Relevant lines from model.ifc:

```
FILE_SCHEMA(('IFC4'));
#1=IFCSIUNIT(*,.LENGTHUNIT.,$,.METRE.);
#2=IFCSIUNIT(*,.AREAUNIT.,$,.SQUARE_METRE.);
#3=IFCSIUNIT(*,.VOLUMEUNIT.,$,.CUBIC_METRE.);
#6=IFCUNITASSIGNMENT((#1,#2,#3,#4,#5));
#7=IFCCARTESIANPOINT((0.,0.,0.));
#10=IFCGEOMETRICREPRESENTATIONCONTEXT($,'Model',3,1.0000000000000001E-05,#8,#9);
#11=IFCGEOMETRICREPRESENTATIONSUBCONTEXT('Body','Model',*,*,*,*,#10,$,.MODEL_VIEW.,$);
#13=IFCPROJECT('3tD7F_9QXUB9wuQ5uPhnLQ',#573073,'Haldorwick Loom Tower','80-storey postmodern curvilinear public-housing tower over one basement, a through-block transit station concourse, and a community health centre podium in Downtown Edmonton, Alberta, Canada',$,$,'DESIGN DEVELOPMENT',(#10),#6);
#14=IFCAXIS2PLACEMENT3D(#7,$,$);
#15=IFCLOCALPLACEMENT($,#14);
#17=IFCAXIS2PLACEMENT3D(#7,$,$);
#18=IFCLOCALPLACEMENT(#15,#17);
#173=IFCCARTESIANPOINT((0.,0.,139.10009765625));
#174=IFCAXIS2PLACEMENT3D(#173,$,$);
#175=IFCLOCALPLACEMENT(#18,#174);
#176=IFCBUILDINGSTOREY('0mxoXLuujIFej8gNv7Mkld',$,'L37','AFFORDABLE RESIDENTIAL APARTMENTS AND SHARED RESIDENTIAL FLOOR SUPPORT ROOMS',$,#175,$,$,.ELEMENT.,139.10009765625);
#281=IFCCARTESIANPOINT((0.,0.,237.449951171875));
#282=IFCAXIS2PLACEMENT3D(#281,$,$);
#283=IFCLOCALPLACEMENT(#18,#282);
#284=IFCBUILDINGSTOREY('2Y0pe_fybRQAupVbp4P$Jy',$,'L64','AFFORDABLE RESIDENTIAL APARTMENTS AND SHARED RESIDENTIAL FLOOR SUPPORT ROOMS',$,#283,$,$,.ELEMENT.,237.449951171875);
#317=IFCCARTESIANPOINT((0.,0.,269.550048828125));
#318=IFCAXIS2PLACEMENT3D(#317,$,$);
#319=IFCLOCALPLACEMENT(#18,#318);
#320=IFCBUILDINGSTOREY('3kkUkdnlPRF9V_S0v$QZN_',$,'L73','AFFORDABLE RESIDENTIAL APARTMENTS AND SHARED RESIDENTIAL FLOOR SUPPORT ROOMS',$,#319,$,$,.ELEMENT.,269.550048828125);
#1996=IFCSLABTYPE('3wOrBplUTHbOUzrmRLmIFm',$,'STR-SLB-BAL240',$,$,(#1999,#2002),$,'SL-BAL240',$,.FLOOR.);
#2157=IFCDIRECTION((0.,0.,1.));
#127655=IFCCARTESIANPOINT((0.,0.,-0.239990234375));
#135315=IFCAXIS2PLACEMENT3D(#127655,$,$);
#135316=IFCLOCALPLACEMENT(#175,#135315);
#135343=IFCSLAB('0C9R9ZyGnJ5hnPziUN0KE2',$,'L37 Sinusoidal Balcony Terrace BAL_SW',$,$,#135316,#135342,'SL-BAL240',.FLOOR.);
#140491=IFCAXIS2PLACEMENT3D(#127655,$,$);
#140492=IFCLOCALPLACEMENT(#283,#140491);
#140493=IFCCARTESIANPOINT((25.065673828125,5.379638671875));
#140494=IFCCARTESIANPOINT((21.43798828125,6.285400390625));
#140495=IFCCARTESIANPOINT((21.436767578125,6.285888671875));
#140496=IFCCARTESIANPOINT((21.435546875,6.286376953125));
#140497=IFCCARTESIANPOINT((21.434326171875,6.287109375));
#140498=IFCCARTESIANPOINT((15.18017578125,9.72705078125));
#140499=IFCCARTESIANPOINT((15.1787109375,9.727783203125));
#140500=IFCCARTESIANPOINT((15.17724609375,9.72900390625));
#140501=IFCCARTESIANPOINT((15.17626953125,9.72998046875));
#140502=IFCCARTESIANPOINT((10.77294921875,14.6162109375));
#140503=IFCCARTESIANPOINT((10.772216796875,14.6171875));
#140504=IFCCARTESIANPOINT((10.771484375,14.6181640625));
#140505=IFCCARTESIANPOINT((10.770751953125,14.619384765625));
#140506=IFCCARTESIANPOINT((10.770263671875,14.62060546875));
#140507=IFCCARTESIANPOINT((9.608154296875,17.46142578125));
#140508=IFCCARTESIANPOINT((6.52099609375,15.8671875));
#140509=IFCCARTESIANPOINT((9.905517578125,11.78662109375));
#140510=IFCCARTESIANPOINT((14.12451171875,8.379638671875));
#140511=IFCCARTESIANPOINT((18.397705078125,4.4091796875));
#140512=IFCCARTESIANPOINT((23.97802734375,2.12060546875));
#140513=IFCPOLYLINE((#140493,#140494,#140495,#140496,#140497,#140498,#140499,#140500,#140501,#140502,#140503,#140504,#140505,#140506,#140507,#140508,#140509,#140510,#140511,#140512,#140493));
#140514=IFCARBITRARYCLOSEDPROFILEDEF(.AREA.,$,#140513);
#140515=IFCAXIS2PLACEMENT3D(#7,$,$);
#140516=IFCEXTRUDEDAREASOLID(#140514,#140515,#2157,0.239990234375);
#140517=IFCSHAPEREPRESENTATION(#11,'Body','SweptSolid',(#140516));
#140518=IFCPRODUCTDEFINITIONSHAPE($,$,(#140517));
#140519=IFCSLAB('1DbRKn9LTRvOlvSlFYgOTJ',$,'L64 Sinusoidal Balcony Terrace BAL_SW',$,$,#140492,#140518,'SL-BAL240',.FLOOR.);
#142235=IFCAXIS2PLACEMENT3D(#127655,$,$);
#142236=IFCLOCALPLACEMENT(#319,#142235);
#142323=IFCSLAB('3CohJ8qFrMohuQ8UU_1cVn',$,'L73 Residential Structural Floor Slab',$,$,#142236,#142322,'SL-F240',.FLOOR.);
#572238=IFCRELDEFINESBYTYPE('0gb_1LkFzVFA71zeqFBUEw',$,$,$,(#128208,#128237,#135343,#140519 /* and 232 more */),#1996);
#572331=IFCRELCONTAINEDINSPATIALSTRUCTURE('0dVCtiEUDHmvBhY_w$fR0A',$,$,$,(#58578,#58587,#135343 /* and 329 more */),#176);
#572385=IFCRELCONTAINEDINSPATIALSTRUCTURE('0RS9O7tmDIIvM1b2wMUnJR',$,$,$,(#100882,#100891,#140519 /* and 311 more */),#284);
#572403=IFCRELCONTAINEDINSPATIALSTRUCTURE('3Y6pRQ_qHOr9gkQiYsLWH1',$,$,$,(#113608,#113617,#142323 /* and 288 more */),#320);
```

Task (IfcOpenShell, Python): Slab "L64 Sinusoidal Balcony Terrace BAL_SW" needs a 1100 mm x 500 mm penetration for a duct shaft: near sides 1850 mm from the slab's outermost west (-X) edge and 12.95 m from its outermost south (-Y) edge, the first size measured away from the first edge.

```python
import numpy as np
import ifcopenshell
import ifcopenshell.api.feature
import ifcopenshell.api.geometry
import ifcopenshell.api.root
import ifcopenshell.geom
import ifcopenshell.util.placement
import ifcopenshell.util.representation
import ifcopenshell.util.shape
import ifcopenshell.util.unit

model = ifcopenshell.open("model.ifc")
unit_scale = ifcopenshell.util.unit.calculate_unit_scale(model)
settings = ifcopenshell.geom.settings()


def volume(element):
    """Net volume in cubic metres, openings subtracted."""
    shape = ifcopenshell.geom.create_shape(settings, element)
    return ifcopenshell.util.shape.get_volume(shape.geometry)


slab = model.by_id(140519)
before = volume(slab)

# Extent in the slab's own axes, in metres. The edges named are its -X and -Y sides.
slab_shape = ifcopenshell.geom.create_shape(settings, slab)
vertices = ifcopenshell.util.shape.get_vertices(slab_shape.geometry)
x_min, y_min, bottom = vertices.min(axis=0)
top = vertices[:, 2].max()

opening = ifcopenshell.api.root.create_entity(model, ifc_class="IfcOpeningElement", name="Duct shaft opening", predefined_type="OPENING")
context = ifcopenshell.util.representation.get_context(model, "Model", "Body", "MODEL_VIEW")
width, depth = 1.1, 0.5
outline = [(0.0, 0.0), (width, 0.0), (width, depth), (0.0, depth), (0.0, 0.0)]
# Overshoot both faces by 50 mm so the cut is clean.
shape = ifcopenshell.api.geometry.add_slab_representation(
    model, context=context, depth=top - bottom + 0.1, polyline=outline
)
ifcopenshell.api.geometry.assign_representation(model, product=opening, representation=shape)

matrix = ifcopenshell.util.placement.get_local_placement(slab.ObjectPlacement)
matrix[:, 3] = matrix @ np.append(np.array([x_min + 1.85, y_min + 12.95, bottom - 0.05]) / unit_scale, 1.0)
ifcopenshell.api.geometry.edit_object_placement(model, product=opening, matrix=matrix, is_si=False)
ifcopenshell.api.feature.add_feature(model, feature=opening, element=slab)

after = volume(slab)

print(f"slab volume {before:.3f} -> {after:.3f} m3")

model.write("model_v2.ifc")
```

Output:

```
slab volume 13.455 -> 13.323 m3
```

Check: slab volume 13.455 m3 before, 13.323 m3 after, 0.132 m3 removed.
